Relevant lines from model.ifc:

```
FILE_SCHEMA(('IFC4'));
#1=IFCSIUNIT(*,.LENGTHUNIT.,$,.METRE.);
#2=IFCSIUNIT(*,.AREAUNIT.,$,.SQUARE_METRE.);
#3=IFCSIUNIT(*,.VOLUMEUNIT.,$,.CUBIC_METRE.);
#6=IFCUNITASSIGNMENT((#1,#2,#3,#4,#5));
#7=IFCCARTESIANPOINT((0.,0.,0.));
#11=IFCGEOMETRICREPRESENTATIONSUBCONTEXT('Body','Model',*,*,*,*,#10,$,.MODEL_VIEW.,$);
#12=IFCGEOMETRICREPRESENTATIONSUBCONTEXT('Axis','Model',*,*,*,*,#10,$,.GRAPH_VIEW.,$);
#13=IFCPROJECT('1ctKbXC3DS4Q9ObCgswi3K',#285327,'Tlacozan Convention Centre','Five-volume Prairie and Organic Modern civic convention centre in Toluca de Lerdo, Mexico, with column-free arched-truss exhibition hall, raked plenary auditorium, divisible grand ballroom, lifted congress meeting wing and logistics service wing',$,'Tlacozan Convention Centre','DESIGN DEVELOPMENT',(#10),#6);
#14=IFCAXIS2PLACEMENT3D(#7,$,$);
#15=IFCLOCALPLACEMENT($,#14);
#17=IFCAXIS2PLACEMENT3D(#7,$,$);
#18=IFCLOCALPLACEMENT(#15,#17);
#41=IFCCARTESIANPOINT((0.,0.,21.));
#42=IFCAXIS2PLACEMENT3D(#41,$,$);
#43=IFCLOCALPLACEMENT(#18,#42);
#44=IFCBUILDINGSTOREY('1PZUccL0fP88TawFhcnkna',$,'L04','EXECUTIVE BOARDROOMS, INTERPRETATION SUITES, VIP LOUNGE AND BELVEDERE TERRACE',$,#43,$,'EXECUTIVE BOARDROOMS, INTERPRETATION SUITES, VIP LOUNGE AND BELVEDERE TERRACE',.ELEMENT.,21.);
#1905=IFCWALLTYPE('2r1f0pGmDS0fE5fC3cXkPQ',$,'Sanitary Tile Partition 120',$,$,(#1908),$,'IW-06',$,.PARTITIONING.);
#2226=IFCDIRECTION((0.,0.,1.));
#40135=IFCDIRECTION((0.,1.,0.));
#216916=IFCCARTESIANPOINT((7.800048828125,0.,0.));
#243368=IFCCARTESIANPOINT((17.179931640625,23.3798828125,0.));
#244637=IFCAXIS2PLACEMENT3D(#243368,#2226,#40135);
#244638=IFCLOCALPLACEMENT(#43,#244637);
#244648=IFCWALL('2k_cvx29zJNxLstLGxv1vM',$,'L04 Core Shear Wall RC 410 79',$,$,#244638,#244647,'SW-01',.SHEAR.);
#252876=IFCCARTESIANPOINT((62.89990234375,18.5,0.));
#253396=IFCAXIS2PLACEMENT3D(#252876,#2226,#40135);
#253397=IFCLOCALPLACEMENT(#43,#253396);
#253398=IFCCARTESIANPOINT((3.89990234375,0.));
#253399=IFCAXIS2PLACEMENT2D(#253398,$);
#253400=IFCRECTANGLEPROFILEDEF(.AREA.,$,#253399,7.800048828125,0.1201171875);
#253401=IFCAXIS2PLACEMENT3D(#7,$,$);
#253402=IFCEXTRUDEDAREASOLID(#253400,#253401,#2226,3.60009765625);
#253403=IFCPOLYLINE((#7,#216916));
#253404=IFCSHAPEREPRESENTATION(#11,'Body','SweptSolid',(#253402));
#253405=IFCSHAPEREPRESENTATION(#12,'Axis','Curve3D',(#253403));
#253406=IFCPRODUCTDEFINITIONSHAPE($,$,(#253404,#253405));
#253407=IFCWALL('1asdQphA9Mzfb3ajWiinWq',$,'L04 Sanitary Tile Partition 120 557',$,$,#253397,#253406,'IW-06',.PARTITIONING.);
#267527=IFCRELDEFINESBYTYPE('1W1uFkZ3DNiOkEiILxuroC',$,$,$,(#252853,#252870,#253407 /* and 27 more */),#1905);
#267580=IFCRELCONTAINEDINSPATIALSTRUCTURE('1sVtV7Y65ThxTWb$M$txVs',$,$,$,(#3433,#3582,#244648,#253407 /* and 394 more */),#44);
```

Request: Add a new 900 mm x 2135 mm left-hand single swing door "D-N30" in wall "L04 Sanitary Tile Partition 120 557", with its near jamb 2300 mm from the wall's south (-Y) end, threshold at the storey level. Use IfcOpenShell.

```python
import numpy as np
import ifcopenshell
import ifcopenshell.api.feature
import ifcopenshell.api.geometry
import ifcopenshell.api.root
import ifcopenshell.api.spatial
import ifcopenshell.geom
import ifcopenshell.util.element
import ifcopenshell.util.placement
import ifcopenshell.util.representation
import ifcopenshell.util.shape
import ifcopenshell.util.unit

model = ifcopenshell.open("model.ifc")
unit_scale = ifcopenshell.util.unit.calculate_unit_scale(model)
settings = ifcopenshell.geom.settings()


def volume(element):
    """Net volume in cubic metres, openings subtracted."""
    shape = ifcopenshell.geom.create_shape(settings, element)
    return ifcopenshell.util.shape.get_volume(shape.geometry)


wall = model.by_id(253407)
storey = ifcopenshell.util.element.get_container(wall, ifc_class="IfcBuildingStorey")
context = ifcopenshell.util.representation.get_context(model, "Model", "Body", "MODEL_VIEW")
before = volume(wall)

width, height, from_end, sill = 0.9, 2.135, 2.3, 0.0  # metres

# The wall runs along its own X axis, and the end named is its -X end.
wall_shape = ifcopenshell.geom.create_shape(settings, wall)
x, y, z = ifcopenshell.util.shape.get_vertices(wall_shape.geometry).T
start = x.min() + from_end
face, thickness = float(y.min()), float(y.max() - y.min())
wall_matrix = ifcopenshell.util.placement.get_local_placement(wall.ObjectPlacement)
level = ifcopenshell.util.placement.get_local_placement(storey.ObjectPlacement)[2, 3]


def in_wall(x, y):
    """Placement at x, y metres in the wall's axes, at sill height."""
    matrix = wall_matrix.copy()
    matrix[:, 3] = wall_matrix @ np.array([x / unit_scale, y / unit_scale, 0.0, 1.0])
    matrix[2, 3] = level + sill / unit_scale
    return matrix


# Opening: a box that overshoots both wall faces by 50 mm.
opening = ifcopenshell.api.root.create_entity(model, ifc_class="IfcOpeningElement", predefined_type="OPENING")
box = ifcopenshell.api.geometry.add_wall_representation(
    model, context=context, length=width, height=height, thickness=thickness + 0.1
)
ifcopenshell.api.geometry.assign_representation(model, product=opening, representation=box)
ifcopenshell.api.geometry.edit_object_placement(model, product=opening, matrix=in_wall(start, face - 0.05), is_si=False)
ifcopenshell.api.feature.add_feature(model, feature=opening, element=wall)

door = ifcopenshell.api.root.create_entity(model, ifc_class="IfcDoor", name="D-N30", predefined_type="DOOR")
door.OverallWidth, door.OverallHeight = width / unit_scale, height / unit_scale
door.OperationType = "SINGLE_SWING_LEFT"
body = ifcopenshell.api.geometry.add_door_representation(
    model,
    context=context,
    overall_width=door.OverallWidth,
    overall_height=door.OverallHeight,
    operation_type="SINGLE_SWING_LEFT",
    lining_properties={"LiningDepth": thickness / unit_scale, "ThresholdDepth": thickness / unit_scale},
)
ifcopenshell.api.geometry.assign_representation(model, product=door, representation=body)
ifcopenshell.api.spatial.assign_container(model, products=[door], relating_structure=storey)
ifcopenshell.api.feature.add_filling(model, opening=opening, element=door)

# The lining spans the wall, so the door starts at the wall face.
ifcopenshell.api.geometry.edit_object_placement(model, product=door, matrix=in_wall(start, face), is_si=False)

after = volume(wall)

print(f"wall volume {before:.3f} -> {after:.3f} m3")

model.write("model-out.ifc")
```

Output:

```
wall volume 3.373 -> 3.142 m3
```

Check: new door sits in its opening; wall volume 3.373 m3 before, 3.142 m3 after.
